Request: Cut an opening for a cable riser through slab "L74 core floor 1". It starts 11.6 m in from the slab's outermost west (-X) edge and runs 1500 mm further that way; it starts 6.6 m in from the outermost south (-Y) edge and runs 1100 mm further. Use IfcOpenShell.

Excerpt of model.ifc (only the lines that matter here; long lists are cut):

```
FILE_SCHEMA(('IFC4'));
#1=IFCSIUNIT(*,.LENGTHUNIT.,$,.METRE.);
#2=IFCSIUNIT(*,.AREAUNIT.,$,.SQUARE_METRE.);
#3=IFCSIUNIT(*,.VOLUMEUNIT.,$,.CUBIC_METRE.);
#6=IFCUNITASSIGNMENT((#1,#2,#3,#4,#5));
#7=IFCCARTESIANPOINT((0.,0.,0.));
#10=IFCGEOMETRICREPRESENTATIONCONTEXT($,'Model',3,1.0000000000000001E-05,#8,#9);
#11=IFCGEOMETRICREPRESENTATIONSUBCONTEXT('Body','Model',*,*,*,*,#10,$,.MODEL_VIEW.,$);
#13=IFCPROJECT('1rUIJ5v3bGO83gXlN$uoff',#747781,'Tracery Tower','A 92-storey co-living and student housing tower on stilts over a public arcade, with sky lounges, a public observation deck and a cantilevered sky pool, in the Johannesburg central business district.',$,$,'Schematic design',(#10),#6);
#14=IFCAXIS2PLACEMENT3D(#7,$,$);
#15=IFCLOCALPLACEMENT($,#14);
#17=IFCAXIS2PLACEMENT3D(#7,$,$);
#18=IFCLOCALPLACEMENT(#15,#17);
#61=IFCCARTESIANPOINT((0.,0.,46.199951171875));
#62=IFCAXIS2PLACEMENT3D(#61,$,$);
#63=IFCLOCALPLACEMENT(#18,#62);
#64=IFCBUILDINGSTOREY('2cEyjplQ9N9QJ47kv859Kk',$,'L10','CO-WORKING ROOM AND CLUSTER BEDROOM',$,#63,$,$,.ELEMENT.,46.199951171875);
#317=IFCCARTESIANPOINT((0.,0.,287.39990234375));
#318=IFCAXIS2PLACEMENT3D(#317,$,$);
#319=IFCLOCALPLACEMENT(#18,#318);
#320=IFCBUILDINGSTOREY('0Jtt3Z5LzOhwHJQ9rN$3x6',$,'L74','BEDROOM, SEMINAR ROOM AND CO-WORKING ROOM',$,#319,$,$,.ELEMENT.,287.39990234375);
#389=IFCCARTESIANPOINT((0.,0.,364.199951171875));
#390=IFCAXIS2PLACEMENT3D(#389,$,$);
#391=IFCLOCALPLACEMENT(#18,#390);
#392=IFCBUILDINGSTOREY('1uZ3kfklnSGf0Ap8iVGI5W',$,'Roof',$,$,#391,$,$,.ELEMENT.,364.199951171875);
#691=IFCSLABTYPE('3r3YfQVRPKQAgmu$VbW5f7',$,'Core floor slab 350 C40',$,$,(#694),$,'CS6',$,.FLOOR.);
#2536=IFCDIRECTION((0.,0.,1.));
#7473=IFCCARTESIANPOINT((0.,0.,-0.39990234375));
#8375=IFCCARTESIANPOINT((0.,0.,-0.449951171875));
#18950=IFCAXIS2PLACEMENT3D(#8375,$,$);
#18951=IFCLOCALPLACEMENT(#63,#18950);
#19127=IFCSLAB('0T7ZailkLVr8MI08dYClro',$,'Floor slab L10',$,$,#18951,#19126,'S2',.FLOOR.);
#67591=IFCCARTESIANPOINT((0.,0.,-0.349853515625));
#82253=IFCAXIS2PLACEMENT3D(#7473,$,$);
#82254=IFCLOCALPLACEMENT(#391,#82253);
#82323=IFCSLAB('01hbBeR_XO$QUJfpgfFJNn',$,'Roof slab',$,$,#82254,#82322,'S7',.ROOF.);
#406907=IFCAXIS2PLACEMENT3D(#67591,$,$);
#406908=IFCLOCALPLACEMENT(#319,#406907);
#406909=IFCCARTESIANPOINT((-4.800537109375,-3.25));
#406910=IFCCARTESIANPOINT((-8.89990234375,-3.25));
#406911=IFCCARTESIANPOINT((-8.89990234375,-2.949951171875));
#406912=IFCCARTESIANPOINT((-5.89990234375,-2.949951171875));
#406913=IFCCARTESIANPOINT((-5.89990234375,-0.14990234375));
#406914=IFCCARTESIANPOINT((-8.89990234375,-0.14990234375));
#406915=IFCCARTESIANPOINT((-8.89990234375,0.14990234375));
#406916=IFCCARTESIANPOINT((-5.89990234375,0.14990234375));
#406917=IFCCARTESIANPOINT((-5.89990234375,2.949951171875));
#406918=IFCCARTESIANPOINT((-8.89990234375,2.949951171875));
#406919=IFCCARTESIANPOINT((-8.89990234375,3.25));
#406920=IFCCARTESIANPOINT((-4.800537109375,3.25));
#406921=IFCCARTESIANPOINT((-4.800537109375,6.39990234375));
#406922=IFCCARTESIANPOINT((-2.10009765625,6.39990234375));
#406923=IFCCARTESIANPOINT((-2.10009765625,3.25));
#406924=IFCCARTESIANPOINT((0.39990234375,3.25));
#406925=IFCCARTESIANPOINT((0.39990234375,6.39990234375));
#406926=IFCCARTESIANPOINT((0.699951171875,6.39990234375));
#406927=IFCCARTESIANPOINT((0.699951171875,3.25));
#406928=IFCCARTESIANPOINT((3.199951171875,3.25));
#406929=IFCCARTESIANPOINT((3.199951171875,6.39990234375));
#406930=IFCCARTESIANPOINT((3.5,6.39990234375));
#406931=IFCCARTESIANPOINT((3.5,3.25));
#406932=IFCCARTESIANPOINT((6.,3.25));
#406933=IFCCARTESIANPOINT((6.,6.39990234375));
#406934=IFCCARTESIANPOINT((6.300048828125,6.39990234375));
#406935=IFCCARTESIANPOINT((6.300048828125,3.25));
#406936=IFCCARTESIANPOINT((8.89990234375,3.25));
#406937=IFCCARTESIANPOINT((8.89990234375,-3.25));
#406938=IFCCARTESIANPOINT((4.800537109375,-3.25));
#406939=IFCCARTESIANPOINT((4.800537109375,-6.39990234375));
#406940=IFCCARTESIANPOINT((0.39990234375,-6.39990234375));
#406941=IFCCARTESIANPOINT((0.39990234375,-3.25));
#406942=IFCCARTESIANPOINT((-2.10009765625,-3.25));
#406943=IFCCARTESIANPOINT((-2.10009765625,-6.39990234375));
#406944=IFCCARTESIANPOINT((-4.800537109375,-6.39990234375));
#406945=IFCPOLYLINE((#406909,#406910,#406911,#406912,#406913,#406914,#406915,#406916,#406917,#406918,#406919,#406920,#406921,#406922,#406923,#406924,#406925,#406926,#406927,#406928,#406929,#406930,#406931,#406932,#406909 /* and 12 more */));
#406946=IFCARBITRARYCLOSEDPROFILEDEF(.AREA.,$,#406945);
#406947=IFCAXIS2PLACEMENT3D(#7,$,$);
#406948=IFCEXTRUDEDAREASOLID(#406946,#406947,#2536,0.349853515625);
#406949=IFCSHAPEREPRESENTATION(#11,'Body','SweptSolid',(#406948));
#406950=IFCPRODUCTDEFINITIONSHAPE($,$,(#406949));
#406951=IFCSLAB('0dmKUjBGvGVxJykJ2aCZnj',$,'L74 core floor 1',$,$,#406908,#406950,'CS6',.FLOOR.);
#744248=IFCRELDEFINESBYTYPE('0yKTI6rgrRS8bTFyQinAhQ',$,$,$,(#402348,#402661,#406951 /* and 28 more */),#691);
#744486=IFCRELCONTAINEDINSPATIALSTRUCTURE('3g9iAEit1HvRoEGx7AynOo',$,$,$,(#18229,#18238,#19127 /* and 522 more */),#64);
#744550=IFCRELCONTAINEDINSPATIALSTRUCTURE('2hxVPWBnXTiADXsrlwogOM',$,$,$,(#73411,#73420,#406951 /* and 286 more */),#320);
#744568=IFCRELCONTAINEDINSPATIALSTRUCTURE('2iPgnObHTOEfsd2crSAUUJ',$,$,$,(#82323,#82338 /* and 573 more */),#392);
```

```python
import numpy as np
import ifcopenshell
import ifcopenshell.api.feature
import ifcopenshell.api.geometry
import ifcopenshell.api.root
import ifcopenshell.geom
import ifcopenshell.util.placement
import ifcopenshell.util.representation
import ifcopenshell.util.shape
import ifcopenshell.util.unit

model = ifcopenshell.open("model.ifc")
unit_scale = ifcopenshell.util.unit.calculate_unit_scale(model)
settings = ifcopenshell.geom.settings()


def volume(element):
    """Net volume in cubic metres, openings subtracted."""
    shape = ifcopenshell.geom.create_shape(settings, element)
    return ifcopenshell.util.shape.get_volume(shape.geometry)


slab = model.by_guid("0dmKUjBGvGVxJykJ2aCZnj")
before = volume(slab)

# Extent in the slab's own axes, in metres. The edges named are its -X and -Y sides.
slab_shape = ifcopenshell.geom.create_shape(settings, slab)
vertices = ifcopenshell.util.shape.get_vertices(slab_shape.geometry)
x_min, y_min, bottom = vertices.min(axis=0)
top = vertices[:, 2].max()

opening = ifcopenshell.api.root.create_entity(model, ifc_class="IfcOpeningElement", name="Cable riser opening", predefined_type="OPENING")
context = ifcopenshell.util.representation.get_context(model, "Model", "Body", "MODEL_VIEW")
width, depth = 1.5, 1.1
outline = [(0.0, 0.0), (width, 0.0), (width, depth), (0.0, depth), (0.0, 0.0)]
# Overshoot both faces by 50 mm so the cut is clean.
shape = ifcopenshell.api.geometry.add_slab_representation(
    model, context=context, depth=top - bottom + 0.1, polyline=outline
)
ifcopenshell.api.geometry.assign_representation(model, product=opening, representation=shape)

matrix = ifcopenshell.util.placement.get_local_placement(slab.ObjectPlacement)
matrix[:, 3] = matrix @ np.append(np.array([x_min + 11.6, y_min + 6.6, bottom - 0.05]) / unit_scale, 1.0)
ifcopenshell.api.geometry.edit_object_placement(model, product=opening, matrix=matrix, is_si=False)
ifcopenshell.api.feature.add_feature(model, feature=opening, element=slab)

after = volume(slab)

print(f"slab volume {before:.3f} -> {after:.3f} m3")

model.write("model_edited.ifc")
```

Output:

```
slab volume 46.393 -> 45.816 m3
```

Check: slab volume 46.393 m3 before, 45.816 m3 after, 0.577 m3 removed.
